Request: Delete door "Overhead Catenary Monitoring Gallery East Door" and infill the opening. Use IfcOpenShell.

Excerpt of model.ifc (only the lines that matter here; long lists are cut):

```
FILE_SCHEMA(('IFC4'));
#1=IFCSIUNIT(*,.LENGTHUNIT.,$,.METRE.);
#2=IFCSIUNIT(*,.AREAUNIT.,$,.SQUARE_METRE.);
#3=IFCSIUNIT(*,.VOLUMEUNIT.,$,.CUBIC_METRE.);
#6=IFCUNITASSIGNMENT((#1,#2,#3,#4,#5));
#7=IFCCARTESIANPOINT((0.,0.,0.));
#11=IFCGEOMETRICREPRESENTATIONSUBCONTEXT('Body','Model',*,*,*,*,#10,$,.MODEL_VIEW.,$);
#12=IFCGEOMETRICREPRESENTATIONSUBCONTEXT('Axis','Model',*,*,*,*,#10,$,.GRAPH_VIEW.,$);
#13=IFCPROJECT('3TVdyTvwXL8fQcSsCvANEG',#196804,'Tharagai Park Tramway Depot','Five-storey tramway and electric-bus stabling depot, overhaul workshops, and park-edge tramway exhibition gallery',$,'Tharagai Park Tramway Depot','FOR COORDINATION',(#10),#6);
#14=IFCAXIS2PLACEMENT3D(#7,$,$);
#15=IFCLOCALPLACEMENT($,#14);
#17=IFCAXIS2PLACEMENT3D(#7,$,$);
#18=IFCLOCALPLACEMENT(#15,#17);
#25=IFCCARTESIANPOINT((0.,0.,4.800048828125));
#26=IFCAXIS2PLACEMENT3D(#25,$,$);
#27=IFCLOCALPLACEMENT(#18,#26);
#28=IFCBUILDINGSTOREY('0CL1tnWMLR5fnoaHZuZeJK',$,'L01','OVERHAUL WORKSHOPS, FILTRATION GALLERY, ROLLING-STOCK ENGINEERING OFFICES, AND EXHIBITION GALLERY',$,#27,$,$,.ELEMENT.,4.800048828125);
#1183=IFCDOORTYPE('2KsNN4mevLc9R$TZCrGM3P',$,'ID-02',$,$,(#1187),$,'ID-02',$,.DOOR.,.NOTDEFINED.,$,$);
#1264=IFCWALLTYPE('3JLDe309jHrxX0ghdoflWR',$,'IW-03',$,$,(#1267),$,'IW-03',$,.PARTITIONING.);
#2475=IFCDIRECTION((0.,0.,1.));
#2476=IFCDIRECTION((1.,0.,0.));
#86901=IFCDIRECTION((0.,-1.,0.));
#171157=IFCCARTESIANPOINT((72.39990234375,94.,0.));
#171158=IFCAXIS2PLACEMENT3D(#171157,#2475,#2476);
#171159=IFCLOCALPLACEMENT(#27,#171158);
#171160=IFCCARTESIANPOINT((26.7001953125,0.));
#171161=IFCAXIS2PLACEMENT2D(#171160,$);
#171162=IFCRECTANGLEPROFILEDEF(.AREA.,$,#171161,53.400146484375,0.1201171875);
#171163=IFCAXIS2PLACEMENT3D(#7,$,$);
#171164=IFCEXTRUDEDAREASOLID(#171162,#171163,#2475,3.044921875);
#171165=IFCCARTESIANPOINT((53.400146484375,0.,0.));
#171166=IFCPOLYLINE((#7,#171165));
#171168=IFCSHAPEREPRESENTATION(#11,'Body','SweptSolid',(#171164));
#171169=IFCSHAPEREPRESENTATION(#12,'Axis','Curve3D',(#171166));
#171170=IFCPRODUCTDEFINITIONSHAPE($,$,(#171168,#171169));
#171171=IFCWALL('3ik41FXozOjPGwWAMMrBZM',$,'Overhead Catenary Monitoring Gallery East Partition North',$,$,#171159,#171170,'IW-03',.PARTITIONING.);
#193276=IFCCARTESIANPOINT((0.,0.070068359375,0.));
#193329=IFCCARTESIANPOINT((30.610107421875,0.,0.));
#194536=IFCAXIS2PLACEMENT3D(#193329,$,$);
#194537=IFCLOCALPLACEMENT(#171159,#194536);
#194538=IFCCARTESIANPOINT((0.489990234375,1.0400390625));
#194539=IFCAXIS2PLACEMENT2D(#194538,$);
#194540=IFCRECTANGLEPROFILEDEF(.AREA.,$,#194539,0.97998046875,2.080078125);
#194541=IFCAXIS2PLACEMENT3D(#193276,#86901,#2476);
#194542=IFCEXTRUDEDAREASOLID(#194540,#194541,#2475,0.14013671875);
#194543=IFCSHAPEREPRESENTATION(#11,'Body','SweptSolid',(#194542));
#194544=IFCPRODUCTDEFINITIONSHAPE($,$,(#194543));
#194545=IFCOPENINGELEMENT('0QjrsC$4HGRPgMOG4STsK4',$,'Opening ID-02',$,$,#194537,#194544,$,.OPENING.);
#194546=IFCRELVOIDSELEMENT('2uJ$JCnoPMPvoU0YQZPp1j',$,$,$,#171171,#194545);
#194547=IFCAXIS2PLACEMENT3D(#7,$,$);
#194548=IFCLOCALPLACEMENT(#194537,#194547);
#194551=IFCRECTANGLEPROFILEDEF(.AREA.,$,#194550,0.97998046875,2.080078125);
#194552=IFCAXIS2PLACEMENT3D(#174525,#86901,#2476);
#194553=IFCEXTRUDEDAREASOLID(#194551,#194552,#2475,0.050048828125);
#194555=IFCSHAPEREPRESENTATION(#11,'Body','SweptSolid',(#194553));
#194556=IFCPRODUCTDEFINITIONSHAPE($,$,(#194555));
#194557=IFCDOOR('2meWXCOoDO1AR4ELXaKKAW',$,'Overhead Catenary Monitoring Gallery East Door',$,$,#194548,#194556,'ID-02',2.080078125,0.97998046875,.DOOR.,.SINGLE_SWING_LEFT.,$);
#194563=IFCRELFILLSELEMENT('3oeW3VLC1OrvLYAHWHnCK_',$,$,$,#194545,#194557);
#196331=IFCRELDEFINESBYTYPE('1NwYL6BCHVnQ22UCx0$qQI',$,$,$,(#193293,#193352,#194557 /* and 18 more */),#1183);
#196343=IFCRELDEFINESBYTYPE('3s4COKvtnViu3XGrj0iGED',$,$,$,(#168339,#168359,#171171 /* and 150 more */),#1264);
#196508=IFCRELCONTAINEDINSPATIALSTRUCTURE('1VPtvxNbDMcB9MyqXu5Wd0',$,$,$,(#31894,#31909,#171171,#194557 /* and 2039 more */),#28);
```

```python
import ifcopenshell
import ifcopenshell.api.feature
import ifcopenshell.api.root
import ifcopenshell.geom
import ifcopenshell.util.shape

model = ifcopenshell.open("model.ifc")
settings = ifcopenshell.geom.settings()


def volume(element):
    """Net volume in cubic metres, openings subtracted."""
    shape = ifcopenshell.geom.create_shape(settings, element)
    return ifcopenshell.util.shape.get_volume(shape.geometry)


door = model.by_id(194557)
opening = door.FillsVoids[0].RelatingOpeningElement
wall = opening.VoidsElements[0].RelatingBuildingElement
before = volume(wall)

ifcopenshell.api.root.remove_product(model, product=door)
ifcopenshell.api.feature.remove_feature(model, feature=opening)

after = volume(wall)

print(f"wall volume {before:.3f} -> {after:.3f} m3")

model.write("model_v2.ifc")
```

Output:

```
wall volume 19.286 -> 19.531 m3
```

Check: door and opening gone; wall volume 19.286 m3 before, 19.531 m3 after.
